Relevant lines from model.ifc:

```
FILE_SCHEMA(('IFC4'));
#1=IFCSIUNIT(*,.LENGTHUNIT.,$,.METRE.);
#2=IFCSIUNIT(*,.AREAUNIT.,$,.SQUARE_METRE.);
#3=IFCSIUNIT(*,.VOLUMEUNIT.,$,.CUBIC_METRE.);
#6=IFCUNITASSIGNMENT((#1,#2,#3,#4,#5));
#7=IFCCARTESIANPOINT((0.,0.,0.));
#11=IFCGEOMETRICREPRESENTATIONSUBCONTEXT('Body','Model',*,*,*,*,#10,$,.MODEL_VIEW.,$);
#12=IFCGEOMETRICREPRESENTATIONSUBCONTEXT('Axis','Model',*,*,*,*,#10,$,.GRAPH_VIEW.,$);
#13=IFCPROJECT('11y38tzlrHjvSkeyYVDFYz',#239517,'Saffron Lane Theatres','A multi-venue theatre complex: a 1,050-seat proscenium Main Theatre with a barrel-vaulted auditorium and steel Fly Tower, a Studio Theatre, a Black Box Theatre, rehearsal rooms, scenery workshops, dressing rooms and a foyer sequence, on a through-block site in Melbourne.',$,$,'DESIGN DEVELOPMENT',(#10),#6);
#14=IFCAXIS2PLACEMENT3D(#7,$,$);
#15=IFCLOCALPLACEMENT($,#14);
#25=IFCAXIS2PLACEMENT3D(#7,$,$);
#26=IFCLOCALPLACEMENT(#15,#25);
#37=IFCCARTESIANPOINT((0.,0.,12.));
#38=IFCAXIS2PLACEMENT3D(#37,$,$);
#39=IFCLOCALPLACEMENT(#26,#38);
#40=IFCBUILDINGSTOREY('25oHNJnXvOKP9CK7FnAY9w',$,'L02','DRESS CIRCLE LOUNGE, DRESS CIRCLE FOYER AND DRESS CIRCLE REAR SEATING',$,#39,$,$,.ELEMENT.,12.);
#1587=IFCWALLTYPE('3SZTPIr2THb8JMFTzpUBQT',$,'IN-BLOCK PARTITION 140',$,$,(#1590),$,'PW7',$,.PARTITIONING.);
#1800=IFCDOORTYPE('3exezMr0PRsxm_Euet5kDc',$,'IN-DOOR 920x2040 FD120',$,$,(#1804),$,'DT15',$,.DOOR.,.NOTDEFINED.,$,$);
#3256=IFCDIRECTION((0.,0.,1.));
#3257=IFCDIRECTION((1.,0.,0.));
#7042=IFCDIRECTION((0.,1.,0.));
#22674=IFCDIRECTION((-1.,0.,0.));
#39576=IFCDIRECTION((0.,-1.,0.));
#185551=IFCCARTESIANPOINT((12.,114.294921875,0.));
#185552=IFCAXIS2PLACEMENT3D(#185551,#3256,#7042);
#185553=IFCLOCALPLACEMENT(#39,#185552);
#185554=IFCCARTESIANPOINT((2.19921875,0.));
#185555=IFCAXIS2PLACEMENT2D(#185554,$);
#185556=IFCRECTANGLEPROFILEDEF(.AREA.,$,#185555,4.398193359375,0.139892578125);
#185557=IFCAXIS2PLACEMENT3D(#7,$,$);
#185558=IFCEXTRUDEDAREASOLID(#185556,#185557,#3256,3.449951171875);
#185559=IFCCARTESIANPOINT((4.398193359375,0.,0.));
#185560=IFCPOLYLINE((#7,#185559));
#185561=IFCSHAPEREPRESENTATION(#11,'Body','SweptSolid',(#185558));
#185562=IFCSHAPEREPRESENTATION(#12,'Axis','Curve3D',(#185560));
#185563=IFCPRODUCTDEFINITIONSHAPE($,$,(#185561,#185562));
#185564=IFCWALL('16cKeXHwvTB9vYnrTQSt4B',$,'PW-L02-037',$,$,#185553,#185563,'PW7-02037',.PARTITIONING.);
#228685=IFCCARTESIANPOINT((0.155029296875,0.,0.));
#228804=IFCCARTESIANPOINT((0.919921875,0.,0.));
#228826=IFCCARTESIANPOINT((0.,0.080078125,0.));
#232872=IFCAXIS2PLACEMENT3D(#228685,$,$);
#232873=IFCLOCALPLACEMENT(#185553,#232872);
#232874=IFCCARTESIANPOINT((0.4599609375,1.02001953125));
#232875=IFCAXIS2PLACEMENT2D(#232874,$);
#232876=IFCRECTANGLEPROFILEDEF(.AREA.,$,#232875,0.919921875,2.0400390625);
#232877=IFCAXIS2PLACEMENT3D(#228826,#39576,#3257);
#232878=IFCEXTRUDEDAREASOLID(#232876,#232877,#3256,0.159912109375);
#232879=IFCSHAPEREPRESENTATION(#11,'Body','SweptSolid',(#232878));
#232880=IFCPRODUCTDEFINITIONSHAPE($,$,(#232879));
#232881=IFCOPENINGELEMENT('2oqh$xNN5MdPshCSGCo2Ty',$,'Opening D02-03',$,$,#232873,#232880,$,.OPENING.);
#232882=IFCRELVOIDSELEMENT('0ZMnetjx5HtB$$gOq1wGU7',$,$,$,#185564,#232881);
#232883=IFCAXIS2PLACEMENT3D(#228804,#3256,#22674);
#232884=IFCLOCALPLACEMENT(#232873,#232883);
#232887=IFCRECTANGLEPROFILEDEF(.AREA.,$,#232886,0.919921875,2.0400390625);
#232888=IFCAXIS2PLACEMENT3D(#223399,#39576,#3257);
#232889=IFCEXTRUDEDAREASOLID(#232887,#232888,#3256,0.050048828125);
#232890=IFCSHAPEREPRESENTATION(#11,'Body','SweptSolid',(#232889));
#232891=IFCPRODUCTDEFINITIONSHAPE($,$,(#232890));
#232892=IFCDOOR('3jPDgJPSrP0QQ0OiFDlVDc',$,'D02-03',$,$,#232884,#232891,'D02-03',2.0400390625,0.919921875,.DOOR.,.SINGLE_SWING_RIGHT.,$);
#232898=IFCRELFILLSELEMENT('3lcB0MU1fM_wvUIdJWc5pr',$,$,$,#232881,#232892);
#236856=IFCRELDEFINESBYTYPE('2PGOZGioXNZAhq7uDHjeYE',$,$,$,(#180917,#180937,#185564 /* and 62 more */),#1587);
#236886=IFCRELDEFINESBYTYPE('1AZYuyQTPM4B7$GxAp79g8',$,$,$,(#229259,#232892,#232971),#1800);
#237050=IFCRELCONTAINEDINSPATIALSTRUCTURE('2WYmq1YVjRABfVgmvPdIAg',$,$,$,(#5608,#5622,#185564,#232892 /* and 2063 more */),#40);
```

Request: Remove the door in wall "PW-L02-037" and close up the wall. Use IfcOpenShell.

```python
import ifcopenshell
import ifcopenshell.api.feature
import ifcopenshell.api.root
import ifcopenshell.geom
import ifcopenshell.util.shape

model = ifcopenshell.open("model.ifc")
settings = ifcopenshell.geom.settings()


def volume(element):
    """Net volume in cubic metres, openings subtracted."""
    shape = ifcopenshell.geom.create_shape(settings, element)
    return ifcopenshell.util.shape.get_volume(shape.geometry)


door = model.by_guid("3jPDgJPSrP0QQ0OiFDlVDc")
opening = door.FillsVoids[0].RelatingOpeningElement
wall = opening.VoidsElements[0].RelatingBuildingElement
before = volume(wall)

ifcopenshell.api.root.remove_product(model, product=door)
ifcopenshell.api.feature.remove_feature(model, feature=opening)

after = volume(wall)

print(f"wall volume {before:.3f} -> {after:.3f} m3")

model.write("model_edited.ifc")
```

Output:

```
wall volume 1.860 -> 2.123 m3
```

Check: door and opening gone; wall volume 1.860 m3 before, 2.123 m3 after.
